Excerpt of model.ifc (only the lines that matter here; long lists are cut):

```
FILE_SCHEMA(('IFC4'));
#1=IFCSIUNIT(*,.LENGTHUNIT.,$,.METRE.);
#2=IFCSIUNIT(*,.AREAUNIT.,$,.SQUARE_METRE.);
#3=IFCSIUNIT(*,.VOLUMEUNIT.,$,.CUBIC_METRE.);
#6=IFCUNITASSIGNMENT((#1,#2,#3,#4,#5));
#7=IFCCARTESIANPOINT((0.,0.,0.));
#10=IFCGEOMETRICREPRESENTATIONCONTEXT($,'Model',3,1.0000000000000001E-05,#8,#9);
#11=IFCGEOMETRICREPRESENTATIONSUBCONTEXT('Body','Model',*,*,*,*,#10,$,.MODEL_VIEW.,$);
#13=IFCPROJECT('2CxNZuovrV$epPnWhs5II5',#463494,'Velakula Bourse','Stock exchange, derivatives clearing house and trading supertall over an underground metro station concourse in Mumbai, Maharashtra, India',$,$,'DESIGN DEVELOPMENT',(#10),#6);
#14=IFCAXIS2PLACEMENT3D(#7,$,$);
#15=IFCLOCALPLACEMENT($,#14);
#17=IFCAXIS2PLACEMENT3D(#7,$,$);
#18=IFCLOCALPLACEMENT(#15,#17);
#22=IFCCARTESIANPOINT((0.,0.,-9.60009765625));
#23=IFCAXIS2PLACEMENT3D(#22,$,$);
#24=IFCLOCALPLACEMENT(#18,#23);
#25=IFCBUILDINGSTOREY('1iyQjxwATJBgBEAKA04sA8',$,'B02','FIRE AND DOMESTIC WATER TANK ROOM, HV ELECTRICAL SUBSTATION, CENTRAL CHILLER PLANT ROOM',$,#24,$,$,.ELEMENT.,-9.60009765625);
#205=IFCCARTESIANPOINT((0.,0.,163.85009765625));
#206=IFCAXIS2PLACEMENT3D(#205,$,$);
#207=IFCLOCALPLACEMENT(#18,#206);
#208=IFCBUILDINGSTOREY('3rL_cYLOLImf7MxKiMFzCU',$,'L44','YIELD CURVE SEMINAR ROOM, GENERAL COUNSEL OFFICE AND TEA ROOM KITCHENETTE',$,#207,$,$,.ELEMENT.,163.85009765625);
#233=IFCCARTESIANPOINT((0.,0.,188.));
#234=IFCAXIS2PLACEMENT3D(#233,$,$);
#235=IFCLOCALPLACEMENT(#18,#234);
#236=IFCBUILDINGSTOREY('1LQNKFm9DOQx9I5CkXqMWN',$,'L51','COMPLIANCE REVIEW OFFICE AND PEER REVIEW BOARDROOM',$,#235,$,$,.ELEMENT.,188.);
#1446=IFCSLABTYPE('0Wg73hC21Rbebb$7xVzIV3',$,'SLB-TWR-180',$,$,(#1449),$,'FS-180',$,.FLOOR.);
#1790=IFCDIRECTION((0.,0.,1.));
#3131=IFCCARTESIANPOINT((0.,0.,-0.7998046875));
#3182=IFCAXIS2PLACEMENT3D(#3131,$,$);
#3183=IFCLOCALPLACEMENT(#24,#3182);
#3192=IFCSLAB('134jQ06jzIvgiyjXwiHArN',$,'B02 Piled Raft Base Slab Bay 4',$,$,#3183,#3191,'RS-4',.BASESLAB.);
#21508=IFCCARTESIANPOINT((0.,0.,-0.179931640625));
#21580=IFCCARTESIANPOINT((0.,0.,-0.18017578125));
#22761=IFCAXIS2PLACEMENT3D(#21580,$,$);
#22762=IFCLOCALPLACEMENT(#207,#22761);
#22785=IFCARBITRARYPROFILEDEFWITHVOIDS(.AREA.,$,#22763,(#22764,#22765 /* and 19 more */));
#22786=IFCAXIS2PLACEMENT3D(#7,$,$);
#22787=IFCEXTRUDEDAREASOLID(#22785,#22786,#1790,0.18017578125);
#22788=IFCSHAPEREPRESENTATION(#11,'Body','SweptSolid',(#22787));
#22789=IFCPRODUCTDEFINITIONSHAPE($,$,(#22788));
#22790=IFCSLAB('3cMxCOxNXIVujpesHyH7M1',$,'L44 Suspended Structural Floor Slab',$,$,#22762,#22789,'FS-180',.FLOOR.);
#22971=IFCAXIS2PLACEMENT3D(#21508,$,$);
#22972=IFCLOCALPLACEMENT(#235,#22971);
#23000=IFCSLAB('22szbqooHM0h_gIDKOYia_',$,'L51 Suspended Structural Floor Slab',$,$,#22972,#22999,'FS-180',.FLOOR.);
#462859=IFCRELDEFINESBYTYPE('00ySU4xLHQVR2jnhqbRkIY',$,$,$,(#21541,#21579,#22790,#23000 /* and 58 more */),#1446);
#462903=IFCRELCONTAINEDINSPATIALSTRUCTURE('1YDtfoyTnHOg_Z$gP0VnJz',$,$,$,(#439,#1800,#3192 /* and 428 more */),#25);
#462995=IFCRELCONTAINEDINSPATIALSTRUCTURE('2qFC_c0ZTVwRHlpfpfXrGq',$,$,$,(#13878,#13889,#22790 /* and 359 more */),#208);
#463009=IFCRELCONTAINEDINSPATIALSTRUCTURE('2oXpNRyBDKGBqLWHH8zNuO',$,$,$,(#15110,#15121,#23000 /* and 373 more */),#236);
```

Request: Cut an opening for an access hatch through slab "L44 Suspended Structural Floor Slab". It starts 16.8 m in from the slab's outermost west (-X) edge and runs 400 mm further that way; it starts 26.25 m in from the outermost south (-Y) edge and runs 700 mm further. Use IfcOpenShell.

```python
import numpy as np
import ifcopenshell
import ifcopenshell.api.feature
import ifcopenshell.api.geometry
import ifcopenshell.api.root
import ifcopenshell.geom
import ifcopenshell.util.placement
import ifcopenshell.util.representation
import ifcopenshell.util.shape
import ifcopenshell.util.unit

model = ifcopenshell.open("model.ifc")
unit_scale = ifcopenshell.util.unit.calculate_unit_scale(model)
settings = ifcopenshell.geom.settings()


def volume(element):
    """Net volume in cubic metres, openings subtracted."""
    shape = ifcopenshell.geom.create_shape(settings, element)
    return ifcopenshell.util.shape.get_volume(shape.geometry)


slab = model.by_guid("3cMxCOxNXIVujpesHyH7M1")
before = volume(slab)

# Extent in the slab's own axes, in metres. The edges named are its -X and -Y sides.
slab_shape = ifcopenshell.geom.create_shape(settings, slab)
vertices = ifcopenshell.util.shape.get_vertices(slab_shape.geometry)
x_min, y_min, bottom = vertices.min(axis=0)
top = vertices[:, 2].max()

opening = ifcopenshell.api.root.create_entity(model, ifc_class="IfcOpeningElement", name="Access hatch opening", predefined_type="OPENING")
context = ifcopenshell.util.representation.get_context(model, "Model", "Body", "MODEL_VIEW")
width, depth = 0.4, 0.7
outline = [(0.0, 0.0), (width, 0.0), (width, depth), (0.0, depth), (0.0, 0.0)]
# Overshoot both faces by 50 mm so the cut is clean.
shape = ifcopenshell.api.geometry.add_slab_representation(
    model, context=context, depth=top - bottom + 0.1, polyline=outline
)
ifcopenshell.api.geometry.assign_representation(model, product=opening, representation=shape)

matrix = ifcopenshell.util.placement.get_local_placement(slab.ObjectPlacement)
matrix[:, 3] = matrix @ np.append(np.array([x_min + 16.8, y_min + 26.25, bottom - 0.05]) / unit_scale, 1.0)
ifcopenshell.api.geometry.edit_object_placement(model, product=opening, matrix=matrix, is_si=False)
ifcopenshell.api.feature.add_feature(model, feature=opening, element=slab)

after = volume(slab)

print(f"slab volume {before:.3f} -> {after:.3f} m3")

model.write("model_edited.ifc")
```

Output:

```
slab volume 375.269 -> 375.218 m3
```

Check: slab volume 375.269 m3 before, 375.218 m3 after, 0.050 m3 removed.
